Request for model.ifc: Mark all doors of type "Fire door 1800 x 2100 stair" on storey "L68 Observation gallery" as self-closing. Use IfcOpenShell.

First a look at what the model holds.

```python
import ifcopenshell
import ifcopenshell.util.element

model = ifcopenshell.open("model.ifc")
print(model.schema)
storey = next(s for s in model.by_type("IfcBuildingStorey") if s.Name == "L68 Observation gallery")
doors = [e for e in ifcopenshell.util.element.get_decomposition(storey) if e.is_a("IfcDoor")]
seen = {}
for e in doors:
    element_type = ifcopenshell.util.element.get_type(e)
    key = (element_type.Name if element_type != e and element_type else None, ifcopenshell.util.element.get_pset(e, "Pset_DoorCommon", "SelfClosing"))
    seen[key] = seen.get(key, 0) + 1
for (name, value), count in sorted(seen.items(), key=str):
    print(count, "x", name, "|", value)
```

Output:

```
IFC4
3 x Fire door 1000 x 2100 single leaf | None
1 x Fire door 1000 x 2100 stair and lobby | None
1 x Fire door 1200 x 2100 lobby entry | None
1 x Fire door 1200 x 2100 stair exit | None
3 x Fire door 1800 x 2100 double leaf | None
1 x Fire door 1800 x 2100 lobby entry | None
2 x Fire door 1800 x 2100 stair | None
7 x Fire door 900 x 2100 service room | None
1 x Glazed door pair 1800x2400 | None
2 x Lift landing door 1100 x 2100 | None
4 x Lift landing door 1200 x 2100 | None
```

```python
import ifcopenshell
import ifcopenshell.api.pset
import ifcopenshell.util.element

model = ifcopenshell.open("model.ifc")

storey = next(s for s in model.by_type("IfcBuildingStorey") if s.Name == "L68 Observation gallery")
doors = [e for e in ifcopenshell.util.element.get_decomposition(storey) if e.is_a("IfcDoor")]

count = 0
for e in doors:
    element_type = ifcopenshell.util.element.get_type(e)
    if element_type in (None, e) or element_type.Name != "Fire door 1800 x 2100 stair":
        continue
    found = ifcopenshell.util.element.get_pset(e, "Pset_DoorCommon", should_inherit=False)
    if found:
        pset = model.by_id(found["id"])
        if len(ifcopenshell.util.element.get_elements_by_pset(pset)) > 1:
            pset = ifcopenshell.api.pset.unshare_pset(model, products=[e], pset=pset)[0]
    else:
        pset = ifcopenshell.api.pset.add_pset(model, product=e, name="Pset_DoorCommon")
    ifcopenshell.api.pset.edit_pset(model, pset=pset, properties={"SelfClosing": True})
    count += 1

print(count, "doors updated")

model.write("model_edited.ifc")
```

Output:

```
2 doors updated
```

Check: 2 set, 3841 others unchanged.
